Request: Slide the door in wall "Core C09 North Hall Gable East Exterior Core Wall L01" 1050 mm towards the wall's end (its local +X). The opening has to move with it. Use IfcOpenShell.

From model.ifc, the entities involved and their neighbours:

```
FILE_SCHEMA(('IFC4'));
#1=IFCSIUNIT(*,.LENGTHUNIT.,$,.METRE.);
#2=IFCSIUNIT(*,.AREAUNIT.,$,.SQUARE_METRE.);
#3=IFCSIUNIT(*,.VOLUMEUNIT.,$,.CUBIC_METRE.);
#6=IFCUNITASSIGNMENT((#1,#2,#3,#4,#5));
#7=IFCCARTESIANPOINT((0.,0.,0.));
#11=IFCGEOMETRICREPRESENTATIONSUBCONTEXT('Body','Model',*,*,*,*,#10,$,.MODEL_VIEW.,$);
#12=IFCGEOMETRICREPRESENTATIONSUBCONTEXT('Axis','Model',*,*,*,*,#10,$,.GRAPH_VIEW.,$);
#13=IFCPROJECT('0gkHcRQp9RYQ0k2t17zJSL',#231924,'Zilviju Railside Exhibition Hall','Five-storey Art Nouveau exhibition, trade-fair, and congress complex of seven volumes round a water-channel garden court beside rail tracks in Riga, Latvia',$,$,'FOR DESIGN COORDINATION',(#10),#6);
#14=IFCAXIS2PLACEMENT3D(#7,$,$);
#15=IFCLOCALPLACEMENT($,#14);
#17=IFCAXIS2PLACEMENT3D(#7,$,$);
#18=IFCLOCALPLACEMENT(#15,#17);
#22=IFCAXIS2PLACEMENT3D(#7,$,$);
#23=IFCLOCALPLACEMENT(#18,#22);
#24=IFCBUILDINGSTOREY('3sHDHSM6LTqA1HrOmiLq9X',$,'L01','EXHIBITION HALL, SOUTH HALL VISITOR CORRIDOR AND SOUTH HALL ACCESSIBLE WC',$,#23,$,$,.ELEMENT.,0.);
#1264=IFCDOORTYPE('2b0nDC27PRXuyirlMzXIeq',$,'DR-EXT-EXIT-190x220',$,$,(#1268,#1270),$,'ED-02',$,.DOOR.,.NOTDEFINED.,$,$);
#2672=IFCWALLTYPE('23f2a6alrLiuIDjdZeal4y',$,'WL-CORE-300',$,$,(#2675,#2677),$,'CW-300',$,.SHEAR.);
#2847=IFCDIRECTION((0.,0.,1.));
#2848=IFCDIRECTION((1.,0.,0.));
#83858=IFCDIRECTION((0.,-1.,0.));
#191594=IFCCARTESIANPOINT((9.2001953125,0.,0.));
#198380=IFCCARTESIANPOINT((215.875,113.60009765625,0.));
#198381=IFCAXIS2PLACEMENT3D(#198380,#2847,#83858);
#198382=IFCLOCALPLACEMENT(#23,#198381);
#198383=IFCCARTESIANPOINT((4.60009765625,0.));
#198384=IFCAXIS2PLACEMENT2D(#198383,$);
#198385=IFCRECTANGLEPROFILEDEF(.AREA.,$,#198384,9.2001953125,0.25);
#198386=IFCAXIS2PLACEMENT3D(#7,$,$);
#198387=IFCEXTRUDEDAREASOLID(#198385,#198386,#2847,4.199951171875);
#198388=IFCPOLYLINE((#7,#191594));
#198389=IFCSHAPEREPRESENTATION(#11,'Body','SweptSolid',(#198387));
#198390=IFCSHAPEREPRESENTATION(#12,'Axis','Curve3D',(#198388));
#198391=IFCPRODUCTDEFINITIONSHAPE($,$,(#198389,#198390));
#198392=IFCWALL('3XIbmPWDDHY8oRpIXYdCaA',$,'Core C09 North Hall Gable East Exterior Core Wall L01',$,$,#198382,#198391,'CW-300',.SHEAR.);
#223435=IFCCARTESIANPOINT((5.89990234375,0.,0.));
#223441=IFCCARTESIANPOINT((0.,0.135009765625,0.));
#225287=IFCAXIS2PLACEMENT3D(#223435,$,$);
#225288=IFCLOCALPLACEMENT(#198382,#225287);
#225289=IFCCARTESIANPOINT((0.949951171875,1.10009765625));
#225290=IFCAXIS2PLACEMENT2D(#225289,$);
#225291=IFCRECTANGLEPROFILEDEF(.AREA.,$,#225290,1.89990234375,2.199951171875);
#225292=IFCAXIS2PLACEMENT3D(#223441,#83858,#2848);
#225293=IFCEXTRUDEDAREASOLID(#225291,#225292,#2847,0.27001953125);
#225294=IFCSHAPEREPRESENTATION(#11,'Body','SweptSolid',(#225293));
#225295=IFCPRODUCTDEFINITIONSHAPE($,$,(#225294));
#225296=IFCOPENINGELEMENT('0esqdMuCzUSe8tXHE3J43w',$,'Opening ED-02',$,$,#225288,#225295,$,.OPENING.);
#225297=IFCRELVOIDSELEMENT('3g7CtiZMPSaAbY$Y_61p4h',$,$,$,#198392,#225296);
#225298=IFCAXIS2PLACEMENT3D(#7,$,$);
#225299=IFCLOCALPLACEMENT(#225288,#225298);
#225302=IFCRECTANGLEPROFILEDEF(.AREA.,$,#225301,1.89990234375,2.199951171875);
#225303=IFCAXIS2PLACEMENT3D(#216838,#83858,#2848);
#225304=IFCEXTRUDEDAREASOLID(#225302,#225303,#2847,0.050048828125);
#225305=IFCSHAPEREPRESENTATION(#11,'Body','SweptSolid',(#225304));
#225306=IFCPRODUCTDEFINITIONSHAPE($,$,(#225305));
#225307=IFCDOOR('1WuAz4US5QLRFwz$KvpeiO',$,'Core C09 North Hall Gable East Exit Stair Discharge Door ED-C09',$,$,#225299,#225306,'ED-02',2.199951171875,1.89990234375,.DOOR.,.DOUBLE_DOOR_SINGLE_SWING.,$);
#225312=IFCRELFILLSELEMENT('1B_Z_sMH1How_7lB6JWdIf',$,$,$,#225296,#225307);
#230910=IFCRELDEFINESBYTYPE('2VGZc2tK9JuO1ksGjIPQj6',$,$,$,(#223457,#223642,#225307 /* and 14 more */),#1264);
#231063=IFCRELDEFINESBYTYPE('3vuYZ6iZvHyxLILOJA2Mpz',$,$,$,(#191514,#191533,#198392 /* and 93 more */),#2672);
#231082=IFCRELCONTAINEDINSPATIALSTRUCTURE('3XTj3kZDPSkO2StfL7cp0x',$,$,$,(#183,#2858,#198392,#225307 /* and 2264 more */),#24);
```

```python
import ifcopenshell
import ifcopenshell.api.geometry
import ifcopenshell.util.placement
import ifcopenshell.util.unit

model = ifcopenshell.open("model.ifc")
unit_scale = ifcopenshell.util.unit.calculate_unit_scale(model)

door = model.by_guid("1WuAz4US5QLRFwz$KvpeiO")
opening = door.FillsVoids[0].RelatingOpeningElement
wall = opening.VoidsElements[0].RelatingBuildingElement

wall_matrix = ifcopenshell.util.placement.get_local_placement(wall.ObjectPlacement)
shift = wall_matrix[:3, 0] * 1.05 / unit_scale
before = ifcopenshell.util.placement.get_local_placement(door.ObjectPlacement)[:3, 3].copy()

# The door is placed relative to its opening, so it follows when the opening moves.
matrix = ifcopenshell.util.placement.get_local_placement(opening.ObjectPlacement)
matrix[:3, 3] += shift
ifcopenshell.api.geometry.edit_object_placement(
    model, product=opening, matrix=matrix, is_si=False, should_transform_children=True
)

after = ifcopenshell.util.placement.get_local_placement(door.ObjectPlacement)[:3, 3]
print("door moved by", (after - before).round(3) + 0.0)

model.write("model_rev.ifc")
```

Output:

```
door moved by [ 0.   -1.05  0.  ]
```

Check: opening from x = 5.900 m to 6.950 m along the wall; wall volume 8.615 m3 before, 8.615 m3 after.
